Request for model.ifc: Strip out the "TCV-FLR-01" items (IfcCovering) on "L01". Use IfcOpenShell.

First a look at what the model holds.

```python
import ifcopenshell
import ifcopenshell.util.element

model = ifcopenshell.open("model.ifc")
print(model.schema)
storey = next(s for s in model.by_type("IfcBuildingStorey") if s.Name == "L01")
coverings = [e for e in ifcopenshell.util.element.get_decomposition(storey) if e.is_a("IfcCovering")]
seen = {}
for e in coverings:
    element_type = ifcopenshell.util.element.get_type(e)
    name = element_type.Name if element_type not in (None, e) else None
    seen[name] = seen.get(name, 0) + 1
for name, count in sorted(seen.items(), key=str):
    print(count, "x", name)
```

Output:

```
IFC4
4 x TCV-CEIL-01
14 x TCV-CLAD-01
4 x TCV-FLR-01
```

```python
import ifcopenshell
import ifcopenshell.api.root
import ifcopenshell.util.element

model = ifcopenshell.open("model.ifc")

storey = next(s for s in model.by_type("IfcBuildingStorey") if s.Name == "L01")
coverings = [e for e in ifcopenshell.util.element.get_decomposition(storey) if e.is_a("IfcCovering")]
targets = [e for e in coverings if (t := ifcopenshell.util.element.get_type(e)) not in (None, e) and t.Name == "TCV-FLR-01"]

for e in targets:
    ifcopenshell.api.root.remove_product(model, product=e)
print(len(targets), "removed")

model.write("model_updated.ifc")
```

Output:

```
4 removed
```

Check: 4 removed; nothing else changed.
